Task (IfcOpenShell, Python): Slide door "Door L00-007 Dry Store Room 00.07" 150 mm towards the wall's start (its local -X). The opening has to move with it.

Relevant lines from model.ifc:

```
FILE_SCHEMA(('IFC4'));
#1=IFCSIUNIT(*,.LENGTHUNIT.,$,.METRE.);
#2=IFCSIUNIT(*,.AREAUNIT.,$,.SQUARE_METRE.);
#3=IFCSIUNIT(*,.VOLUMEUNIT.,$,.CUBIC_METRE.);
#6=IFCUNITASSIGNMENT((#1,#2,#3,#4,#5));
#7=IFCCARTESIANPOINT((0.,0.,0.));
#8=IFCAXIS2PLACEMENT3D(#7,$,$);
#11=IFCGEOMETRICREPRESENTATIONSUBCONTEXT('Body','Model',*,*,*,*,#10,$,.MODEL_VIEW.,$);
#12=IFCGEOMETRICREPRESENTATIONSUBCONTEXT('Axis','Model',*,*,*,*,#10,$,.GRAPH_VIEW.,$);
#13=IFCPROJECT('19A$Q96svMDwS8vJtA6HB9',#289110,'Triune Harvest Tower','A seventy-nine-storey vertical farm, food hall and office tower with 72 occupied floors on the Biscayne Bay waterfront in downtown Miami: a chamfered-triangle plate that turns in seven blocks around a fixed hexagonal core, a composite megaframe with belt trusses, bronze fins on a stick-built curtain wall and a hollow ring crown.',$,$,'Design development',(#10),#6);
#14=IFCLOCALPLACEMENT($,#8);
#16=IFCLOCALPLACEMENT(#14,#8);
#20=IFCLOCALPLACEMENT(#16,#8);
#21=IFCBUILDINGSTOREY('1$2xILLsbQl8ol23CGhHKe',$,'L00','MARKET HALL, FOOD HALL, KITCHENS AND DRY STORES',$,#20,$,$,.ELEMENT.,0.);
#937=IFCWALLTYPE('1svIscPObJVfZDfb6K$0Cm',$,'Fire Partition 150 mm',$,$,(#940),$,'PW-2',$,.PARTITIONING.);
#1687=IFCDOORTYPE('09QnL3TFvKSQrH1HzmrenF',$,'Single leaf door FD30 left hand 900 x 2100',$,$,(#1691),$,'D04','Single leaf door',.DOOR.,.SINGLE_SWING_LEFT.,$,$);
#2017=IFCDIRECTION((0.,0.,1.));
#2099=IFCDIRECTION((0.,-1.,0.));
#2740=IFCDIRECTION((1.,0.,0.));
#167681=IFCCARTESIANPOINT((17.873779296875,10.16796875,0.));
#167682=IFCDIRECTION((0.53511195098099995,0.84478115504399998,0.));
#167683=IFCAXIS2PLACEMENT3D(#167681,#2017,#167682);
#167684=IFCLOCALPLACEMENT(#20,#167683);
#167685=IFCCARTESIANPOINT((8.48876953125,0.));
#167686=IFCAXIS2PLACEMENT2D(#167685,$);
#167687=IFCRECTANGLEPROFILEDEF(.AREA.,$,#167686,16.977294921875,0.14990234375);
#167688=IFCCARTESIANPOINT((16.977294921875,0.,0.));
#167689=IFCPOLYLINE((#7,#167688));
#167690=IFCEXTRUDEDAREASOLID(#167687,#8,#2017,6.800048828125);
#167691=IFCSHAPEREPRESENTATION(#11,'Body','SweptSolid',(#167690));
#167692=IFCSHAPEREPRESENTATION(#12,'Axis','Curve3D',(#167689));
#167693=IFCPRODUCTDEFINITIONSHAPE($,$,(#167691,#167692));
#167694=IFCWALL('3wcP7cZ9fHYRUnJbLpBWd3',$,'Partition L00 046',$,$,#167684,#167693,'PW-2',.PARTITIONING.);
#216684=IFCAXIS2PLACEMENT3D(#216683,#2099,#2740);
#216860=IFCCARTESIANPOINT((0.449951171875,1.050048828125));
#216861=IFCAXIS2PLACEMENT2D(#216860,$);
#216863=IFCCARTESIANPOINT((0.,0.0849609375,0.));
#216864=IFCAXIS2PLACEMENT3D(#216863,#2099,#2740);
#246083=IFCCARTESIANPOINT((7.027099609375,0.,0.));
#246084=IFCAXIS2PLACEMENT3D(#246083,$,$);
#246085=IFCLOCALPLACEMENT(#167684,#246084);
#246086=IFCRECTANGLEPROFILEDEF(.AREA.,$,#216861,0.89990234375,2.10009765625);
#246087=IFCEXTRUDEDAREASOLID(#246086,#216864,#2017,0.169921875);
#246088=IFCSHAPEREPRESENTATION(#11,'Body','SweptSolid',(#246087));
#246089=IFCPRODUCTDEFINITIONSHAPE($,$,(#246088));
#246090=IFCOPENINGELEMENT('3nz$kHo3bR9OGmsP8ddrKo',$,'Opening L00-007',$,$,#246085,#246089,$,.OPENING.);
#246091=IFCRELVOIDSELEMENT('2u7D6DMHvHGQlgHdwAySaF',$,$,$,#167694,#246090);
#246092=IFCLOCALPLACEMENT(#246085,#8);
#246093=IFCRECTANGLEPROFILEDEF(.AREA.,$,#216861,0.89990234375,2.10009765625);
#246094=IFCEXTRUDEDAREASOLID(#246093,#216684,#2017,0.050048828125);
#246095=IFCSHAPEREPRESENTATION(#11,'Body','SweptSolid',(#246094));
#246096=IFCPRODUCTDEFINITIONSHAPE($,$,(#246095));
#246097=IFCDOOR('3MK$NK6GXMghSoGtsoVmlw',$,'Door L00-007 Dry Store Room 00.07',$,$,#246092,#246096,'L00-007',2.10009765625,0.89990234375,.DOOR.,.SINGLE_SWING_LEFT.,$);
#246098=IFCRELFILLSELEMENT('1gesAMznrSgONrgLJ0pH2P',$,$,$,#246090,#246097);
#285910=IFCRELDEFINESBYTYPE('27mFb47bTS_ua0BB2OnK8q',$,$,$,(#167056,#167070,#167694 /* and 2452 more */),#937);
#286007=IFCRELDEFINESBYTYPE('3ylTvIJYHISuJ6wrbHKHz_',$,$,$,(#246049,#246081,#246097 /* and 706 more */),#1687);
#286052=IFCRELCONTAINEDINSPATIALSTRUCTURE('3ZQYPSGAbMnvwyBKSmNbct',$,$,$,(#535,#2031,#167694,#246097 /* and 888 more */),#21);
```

```python
import ifcopenshell
import ifcopenshell.api.geometry
import ifcopenshell.util.placement

model = ifcopenshell.open("model.ifc")

door = model.by_guid("3MK$NK6GXMghSoGtsoVmlw")
opening = door.FillsVoids[0].RelatingOpeningElement
wall = opening.VoidsElements[0].RelatingBuildingElement

wall_matrix = ifcopenshell.util.placement.get_local_placement(wall.ObjectPlacement)
shift = wall_matrix[:3, 0] * -0.15
before = ifcopenshell.util.placement.get_local_placement(door.ObjectPlacement)[:3, 3].copy()

# The door is placed relative to its opening, so it follows when the opening moves.
matrix = ifcopenshell.util.placement.get_local_placement(opening.ObjectPlacement)
matrix[:3, 3] += shift
ifcopenshell.api.geometry.edit_object_placement(
    model, product=opening, matrix=matrix, is_si=False, should_transform_children=True
)

after = ifcopenshell.util.placement.get_local_placement(door.ObjectPlacement)[:3, 3]
print("door moved by", (after - before).round(3) + 0.0)

model.write("model_edited.ifc")
```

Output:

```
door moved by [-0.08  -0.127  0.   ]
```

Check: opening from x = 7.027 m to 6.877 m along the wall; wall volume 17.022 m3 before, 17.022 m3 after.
